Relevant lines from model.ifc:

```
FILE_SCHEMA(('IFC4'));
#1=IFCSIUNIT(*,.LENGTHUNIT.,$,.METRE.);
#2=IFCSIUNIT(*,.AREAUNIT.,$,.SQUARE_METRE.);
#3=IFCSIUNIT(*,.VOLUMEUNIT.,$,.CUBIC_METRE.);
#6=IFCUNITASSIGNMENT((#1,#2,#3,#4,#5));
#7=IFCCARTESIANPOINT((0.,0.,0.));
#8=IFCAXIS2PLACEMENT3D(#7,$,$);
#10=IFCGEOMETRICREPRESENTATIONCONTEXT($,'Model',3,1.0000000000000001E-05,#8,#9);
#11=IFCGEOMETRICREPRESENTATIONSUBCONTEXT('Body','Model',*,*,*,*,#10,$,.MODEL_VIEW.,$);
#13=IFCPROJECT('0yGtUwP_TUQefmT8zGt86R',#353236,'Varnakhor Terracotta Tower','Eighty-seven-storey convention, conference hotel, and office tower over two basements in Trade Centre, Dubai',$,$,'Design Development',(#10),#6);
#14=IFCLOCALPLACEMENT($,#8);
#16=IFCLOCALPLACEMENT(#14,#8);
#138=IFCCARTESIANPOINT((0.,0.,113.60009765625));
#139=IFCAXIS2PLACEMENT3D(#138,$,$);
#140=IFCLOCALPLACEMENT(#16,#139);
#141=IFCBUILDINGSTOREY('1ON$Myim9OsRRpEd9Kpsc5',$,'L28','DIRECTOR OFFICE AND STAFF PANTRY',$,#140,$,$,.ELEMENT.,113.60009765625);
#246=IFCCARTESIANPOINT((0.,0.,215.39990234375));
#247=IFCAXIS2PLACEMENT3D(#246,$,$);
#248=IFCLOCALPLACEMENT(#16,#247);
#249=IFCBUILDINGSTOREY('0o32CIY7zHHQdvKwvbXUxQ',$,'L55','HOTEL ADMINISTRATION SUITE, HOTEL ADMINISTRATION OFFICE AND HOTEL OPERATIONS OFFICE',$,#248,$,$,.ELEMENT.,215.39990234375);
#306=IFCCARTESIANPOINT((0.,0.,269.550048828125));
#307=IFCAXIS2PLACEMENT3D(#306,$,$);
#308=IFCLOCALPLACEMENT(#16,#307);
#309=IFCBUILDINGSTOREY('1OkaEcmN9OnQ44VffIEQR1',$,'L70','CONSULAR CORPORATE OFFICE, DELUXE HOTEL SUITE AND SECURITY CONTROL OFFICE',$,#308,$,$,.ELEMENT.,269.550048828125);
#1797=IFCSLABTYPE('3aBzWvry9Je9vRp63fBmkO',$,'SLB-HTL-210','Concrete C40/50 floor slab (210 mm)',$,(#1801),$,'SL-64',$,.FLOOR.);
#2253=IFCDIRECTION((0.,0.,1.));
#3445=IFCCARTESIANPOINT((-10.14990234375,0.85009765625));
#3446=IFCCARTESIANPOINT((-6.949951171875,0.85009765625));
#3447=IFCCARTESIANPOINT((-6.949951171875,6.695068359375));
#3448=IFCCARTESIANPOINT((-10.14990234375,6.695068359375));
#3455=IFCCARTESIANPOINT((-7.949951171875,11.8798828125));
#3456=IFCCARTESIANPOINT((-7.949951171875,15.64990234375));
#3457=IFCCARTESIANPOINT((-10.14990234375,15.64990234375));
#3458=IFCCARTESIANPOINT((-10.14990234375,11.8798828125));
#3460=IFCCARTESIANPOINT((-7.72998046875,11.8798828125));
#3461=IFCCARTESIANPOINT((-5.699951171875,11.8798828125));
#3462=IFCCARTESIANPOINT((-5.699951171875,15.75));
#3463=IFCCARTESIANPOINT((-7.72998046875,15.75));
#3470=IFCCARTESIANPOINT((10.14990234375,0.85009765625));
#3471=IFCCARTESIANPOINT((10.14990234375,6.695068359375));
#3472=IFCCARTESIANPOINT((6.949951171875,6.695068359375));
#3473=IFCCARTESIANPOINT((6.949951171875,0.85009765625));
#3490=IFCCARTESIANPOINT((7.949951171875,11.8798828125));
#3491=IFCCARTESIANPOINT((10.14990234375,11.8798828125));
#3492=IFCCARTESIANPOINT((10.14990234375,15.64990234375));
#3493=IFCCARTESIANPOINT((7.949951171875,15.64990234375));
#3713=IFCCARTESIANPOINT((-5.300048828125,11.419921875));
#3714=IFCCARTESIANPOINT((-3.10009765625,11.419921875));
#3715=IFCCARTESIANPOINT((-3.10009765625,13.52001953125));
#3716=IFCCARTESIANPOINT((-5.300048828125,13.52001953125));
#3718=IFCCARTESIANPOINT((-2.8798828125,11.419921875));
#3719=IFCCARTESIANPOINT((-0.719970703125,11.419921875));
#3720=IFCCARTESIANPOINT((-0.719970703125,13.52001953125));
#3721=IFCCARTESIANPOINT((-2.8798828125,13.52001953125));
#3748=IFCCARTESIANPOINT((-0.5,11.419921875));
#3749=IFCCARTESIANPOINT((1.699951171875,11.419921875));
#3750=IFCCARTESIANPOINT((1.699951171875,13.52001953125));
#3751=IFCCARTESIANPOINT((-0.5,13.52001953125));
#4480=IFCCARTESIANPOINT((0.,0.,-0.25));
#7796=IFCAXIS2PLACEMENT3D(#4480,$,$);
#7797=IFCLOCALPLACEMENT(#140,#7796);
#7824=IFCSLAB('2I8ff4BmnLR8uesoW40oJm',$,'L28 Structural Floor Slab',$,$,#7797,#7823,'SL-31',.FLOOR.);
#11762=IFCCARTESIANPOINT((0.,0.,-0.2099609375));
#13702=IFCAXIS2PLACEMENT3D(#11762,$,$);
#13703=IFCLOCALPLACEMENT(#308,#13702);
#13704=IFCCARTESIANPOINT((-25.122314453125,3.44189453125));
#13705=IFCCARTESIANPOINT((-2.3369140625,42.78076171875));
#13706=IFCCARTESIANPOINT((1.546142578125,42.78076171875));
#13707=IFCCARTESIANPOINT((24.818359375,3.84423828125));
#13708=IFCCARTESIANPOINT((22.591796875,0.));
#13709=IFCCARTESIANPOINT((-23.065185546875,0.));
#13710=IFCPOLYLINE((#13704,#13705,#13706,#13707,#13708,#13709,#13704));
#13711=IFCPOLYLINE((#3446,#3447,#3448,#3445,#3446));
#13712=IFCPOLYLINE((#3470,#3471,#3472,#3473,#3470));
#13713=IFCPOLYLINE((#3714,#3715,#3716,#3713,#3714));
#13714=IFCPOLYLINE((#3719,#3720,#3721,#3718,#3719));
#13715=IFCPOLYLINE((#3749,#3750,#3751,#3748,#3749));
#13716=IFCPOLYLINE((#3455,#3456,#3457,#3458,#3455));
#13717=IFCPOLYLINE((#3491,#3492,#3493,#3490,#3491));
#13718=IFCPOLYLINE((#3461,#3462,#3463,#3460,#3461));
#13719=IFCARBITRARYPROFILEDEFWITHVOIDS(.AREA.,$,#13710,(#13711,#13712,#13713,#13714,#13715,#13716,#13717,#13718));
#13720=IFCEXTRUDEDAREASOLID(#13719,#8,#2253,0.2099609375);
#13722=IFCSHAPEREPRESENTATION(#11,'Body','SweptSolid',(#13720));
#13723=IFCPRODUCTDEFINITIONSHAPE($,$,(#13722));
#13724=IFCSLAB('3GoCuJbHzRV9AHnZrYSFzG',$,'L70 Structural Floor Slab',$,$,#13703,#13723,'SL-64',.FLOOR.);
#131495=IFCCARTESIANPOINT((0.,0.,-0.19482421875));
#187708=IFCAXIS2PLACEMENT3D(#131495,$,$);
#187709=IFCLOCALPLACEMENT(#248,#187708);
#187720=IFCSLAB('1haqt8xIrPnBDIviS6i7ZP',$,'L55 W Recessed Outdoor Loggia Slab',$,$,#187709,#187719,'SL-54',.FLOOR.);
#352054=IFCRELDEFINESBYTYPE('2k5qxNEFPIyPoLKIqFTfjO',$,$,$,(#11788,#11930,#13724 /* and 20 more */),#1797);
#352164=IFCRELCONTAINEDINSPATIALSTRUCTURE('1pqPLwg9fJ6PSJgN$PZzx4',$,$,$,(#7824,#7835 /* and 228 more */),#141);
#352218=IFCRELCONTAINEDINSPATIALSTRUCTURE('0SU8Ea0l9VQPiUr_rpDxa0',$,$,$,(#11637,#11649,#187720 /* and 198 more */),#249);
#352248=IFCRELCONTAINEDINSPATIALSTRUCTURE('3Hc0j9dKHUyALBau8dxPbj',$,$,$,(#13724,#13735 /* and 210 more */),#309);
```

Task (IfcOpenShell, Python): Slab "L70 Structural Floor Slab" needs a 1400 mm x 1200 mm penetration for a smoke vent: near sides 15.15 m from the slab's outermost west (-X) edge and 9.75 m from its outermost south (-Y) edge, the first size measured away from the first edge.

```python
import numpy as np
import ifcopenshell
import ifcopenshell.api.feature
import ifcopenshell.api.geometry
import ifcopenshell.api.root
import ifcopenshell.geom
import ifcopenshell.util.placement
import ifcopenshell.util.representation
import ifcopenshell.util.shape
import ifcopenshell.util.unit

model = ifcopenshell.open("model.ifc")
unit_scale = ifcopenshell.util.unit.calculate_unit_scale(model)
settings = ifcopenshell.geom.settings()


def volume(element):
    """Net volume in cubic metres, openings subtracted."""
    shape = ifcopenshell.geom.create_shape(settings, element)
    return ifcopenshell.util.shape.get_volume(shape.geometry)


slab = model.by_id(13724)
before = volume(slab)

# Extent in the slab's own axes, in metres. The edges named are its -X and -Y sides.
slab_shape = ifcopenshell.geom.create_shape(settings, slab)
vertices = ifcopenshell.util.shape.get_vertices(slab_shape.geometry)
x_min, y_min, bottom = vertices.min(axis=0)
top = vertices[:, 2].max()

opening = ifcopenshell.api.root.create_entity(model, ifc_class="IfcOpeningElement", name="Smoke vent opening", predefined_type="OPENING")
context = ifcopenshell.util.representation.get_context(model, "Model", "Body", "MODEL_VIEW")
width, depth = 1.4, 1.2
outline = [(0.0, 0.0), (width, 0.0), (width, depth), (0.0, depth), (0.0, 0.0)]
# Overshoot both faces by 50 mm so the cut is clean.
shape = ifcopenshell.api.geometry.add_slab_representation(
    model, context=context, depth=top - bottom + 0.1, polyline=outline
)
ifcopenshell.api.geometry.assign_representation(model, product=opening, representation=shape)

matrix = ifcopenshell.util.placement.get_local_placement(slab.ObjectPlacement)
matrix[:, 3] = matrix @ np.append(np.array([x_min + 15.15, y_min + 9.75, bottom - 0.05]) / unit_scale, 1.0)
ifcopenshell.api.geometry.edit_object_placement(model, product=opening, matrix=matrix, is_si=False)
ifcopenshell.api.feature.add_feature(model, feature=opening, element=slab)

after = volume(slab)

print(f"slab volume {before:.3f} -> {after:.3f} m3")

model.write("model_edited.ifc")
```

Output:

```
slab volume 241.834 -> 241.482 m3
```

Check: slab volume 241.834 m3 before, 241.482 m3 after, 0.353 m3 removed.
